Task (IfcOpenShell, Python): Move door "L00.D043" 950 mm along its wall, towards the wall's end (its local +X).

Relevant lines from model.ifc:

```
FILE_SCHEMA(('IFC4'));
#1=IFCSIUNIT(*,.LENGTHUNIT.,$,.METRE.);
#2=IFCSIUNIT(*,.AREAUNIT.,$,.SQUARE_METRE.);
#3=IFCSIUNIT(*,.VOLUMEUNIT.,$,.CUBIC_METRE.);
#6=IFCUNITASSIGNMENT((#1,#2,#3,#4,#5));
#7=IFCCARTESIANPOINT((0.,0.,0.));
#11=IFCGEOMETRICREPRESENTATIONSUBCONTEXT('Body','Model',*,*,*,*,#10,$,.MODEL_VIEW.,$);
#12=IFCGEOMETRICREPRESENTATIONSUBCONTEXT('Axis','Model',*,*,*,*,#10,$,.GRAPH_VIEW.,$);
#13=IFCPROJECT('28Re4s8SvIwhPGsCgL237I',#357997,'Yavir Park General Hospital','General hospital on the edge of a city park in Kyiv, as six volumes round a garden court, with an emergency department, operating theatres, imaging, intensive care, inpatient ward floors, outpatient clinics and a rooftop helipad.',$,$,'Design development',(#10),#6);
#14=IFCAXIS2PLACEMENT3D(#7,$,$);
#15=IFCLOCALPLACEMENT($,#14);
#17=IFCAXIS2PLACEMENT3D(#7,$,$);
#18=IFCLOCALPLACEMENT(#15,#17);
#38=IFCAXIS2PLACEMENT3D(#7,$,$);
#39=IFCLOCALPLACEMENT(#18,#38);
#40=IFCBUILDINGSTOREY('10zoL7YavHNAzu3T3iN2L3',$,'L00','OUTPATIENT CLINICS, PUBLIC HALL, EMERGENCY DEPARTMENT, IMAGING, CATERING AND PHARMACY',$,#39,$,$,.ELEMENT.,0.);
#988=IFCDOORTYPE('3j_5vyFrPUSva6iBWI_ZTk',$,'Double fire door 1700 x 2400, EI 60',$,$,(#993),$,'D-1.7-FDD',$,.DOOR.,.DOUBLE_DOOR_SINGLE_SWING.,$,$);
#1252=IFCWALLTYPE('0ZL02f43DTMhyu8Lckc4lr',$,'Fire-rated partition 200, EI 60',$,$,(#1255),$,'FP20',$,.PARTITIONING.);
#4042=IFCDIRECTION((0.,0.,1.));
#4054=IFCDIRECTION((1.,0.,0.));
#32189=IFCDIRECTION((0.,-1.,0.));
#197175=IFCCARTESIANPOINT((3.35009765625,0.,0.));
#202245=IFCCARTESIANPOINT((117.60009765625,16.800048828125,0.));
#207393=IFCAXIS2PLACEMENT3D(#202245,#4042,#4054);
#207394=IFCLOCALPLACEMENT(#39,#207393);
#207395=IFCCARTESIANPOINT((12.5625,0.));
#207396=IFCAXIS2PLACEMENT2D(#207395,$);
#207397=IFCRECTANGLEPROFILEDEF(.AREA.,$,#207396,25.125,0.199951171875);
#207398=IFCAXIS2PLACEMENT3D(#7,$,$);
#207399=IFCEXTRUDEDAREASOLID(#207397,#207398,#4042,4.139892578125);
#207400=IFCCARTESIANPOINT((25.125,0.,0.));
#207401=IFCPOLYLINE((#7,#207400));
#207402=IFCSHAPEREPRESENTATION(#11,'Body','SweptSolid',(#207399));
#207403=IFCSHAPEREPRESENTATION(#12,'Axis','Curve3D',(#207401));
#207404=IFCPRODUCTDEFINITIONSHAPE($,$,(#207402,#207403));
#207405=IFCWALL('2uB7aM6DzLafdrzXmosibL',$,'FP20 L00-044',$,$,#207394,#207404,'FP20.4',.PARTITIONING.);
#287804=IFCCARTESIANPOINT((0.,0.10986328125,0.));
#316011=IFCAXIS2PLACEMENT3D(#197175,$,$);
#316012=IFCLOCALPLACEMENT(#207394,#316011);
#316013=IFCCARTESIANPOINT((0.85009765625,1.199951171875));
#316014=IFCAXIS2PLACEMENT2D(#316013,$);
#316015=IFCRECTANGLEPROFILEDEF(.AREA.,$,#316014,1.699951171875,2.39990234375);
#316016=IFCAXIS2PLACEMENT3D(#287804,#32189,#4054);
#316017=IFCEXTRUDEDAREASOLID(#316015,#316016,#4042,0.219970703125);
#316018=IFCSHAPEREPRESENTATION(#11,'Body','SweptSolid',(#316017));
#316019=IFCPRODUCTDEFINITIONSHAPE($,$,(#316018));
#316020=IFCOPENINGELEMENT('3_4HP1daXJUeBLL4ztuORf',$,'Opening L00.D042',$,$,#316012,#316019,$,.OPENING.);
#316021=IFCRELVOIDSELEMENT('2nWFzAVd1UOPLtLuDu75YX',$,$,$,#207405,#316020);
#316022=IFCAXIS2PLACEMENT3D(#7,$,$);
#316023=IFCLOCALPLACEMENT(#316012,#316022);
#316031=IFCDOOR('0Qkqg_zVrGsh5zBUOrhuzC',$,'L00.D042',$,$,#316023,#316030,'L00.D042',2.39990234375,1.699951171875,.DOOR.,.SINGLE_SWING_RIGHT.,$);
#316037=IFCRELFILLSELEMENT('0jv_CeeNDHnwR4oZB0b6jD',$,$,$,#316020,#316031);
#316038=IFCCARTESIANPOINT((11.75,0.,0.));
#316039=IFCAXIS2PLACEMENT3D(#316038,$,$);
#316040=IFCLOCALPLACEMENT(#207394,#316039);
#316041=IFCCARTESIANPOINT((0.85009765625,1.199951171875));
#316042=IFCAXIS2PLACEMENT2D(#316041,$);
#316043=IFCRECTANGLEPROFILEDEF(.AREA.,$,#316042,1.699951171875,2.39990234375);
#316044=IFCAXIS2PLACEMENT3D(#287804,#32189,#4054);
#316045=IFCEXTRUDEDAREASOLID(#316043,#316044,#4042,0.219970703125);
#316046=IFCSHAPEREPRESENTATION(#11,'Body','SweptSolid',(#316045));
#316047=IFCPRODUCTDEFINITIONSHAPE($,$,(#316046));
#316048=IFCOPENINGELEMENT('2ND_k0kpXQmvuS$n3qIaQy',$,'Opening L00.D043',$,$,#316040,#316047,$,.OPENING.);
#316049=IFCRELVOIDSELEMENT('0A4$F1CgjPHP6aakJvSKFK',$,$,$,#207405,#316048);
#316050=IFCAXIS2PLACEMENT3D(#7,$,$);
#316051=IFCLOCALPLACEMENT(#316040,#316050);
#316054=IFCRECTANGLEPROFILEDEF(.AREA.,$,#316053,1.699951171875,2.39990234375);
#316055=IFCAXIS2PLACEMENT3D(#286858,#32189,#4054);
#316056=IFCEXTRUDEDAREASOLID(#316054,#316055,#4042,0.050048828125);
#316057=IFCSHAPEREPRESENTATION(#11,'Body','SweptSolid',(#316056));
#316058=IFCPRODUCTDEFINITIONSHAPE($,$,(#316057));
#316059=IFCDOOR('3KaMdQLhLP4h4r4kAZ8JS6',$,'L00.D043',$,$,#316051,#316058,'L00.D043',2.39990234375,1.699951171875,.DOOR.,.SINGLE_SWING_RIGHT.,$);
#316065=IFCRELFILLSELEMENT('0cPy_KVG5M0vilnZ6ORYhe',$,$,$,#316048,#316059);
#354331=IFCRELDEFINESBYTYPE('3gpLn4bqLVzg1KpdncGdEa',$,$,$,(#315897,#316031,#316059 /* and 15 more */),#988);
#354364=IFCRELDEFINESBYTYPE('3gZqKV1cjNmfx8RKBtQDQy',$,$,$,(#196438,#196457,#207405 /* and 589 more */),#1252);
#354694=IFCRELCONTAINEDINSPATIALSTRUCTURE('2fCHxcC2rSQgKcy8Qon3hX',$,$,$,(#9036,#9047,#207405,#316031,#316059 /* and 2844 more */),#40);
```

```python
import ifcopenshell
import ifcopenshell.api.geometry
import ifcopenshell.util.placement
import ifcopenshell.util.unit

model = ifcopenshell.open("model.ifc")
unit_scale = ifcopenshell.util.unit.calculate_unit_scale(model)

door = model.by_guid("3KaMdQLhLP4h4r4kAZ8JS6")
opening = door.FillsVoids[0].RelatingOpeningElement
wall = opening.VoidsElements[0].RelatingBuildingElement

wall_matrix = ifcopenshell.util.placement.get_local_placement(wall.ObjectPlacement)
shift = wall_matrix[:3, 0] * 0.95 / unit_scale
before = ifcopenshell.util.placement.get_local_placement(door.ObjectPlacement)[:3, 3].copy()

# The door is placed relative to its opening, so it follows when the opening moves.
matrix = ifcopenshell.util.placement.get_local_placement(opening.ObjectPlacement)
matrix[:3, 3] += shift
ifcopenshell.api.geometry.edit_object_placement(
    model, product=opening, matrix=matrix, is_si=False, should_transform_children=True
)

after = ifcopenshell.util.placement.get_local_placement(door.ObjectPlacement)[:3, 3]
print("door moved by", (after - before).round(3) + 0.0)

model.write("model_v2.ifc")
```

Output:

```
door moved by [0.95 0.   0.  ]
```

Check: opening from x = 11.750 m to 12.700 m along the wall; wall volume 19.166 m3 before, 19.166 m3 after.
